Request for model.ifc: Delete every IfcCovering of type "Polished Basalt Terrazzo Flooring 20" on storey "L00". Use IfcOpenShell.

First a look at what the model holds.

```python
import ifcopenshell
import ifcopenshell.util.element

model = ifcopenshell.open("model.ifc")
print(model.schema)
storey = next(s for s in model.by_type("IfcBuildingStorey") if s.Name == "L00")
coverings = [e for e in ifcopenshell.util.element.get_decomposition(storey) if e.is_a("IfcCovering")]
seen = {}
for e in coverings:
    element_type = ifcopenshell.util.element.get_type(e)
    name = element_type.Name if element_type not in (None, e) else None
    seen[name] = seen.get(name, 0) + 1
for name, count in sorted(seen.items(), key=str):
    print(count, "x", name)
```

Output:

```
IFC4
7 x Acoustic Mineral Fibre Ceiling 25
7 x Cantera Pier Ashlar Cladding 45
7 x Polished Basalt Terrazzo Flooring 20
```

```python
import ifcopenshell
import ifcopenshell.api.root
import ifcopenshell.util.element

model = ifcopenshell.open("model.ifc")

storey = next(s for s in model.by_type("IfcBuildingStorey") if s.Name == "L00")
coverings = [e for e in ifcopenshell.util.element.get_decomposition(storey) if e.is_a("IfcCovering")]
targets = [e for e in coverings if (t := ifcopenshell.util.element.get_type(e)) not in (None, e) and t.Name == "Polished Basalt Terrazzo Flooring 20"]

for e in targets:
    ifcopenshell.api.root.remove_product(model, product=e)
print(len(targets), "removed")

model.write("model_updated.ifc")
```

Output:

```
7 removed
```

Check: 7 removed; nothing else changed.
